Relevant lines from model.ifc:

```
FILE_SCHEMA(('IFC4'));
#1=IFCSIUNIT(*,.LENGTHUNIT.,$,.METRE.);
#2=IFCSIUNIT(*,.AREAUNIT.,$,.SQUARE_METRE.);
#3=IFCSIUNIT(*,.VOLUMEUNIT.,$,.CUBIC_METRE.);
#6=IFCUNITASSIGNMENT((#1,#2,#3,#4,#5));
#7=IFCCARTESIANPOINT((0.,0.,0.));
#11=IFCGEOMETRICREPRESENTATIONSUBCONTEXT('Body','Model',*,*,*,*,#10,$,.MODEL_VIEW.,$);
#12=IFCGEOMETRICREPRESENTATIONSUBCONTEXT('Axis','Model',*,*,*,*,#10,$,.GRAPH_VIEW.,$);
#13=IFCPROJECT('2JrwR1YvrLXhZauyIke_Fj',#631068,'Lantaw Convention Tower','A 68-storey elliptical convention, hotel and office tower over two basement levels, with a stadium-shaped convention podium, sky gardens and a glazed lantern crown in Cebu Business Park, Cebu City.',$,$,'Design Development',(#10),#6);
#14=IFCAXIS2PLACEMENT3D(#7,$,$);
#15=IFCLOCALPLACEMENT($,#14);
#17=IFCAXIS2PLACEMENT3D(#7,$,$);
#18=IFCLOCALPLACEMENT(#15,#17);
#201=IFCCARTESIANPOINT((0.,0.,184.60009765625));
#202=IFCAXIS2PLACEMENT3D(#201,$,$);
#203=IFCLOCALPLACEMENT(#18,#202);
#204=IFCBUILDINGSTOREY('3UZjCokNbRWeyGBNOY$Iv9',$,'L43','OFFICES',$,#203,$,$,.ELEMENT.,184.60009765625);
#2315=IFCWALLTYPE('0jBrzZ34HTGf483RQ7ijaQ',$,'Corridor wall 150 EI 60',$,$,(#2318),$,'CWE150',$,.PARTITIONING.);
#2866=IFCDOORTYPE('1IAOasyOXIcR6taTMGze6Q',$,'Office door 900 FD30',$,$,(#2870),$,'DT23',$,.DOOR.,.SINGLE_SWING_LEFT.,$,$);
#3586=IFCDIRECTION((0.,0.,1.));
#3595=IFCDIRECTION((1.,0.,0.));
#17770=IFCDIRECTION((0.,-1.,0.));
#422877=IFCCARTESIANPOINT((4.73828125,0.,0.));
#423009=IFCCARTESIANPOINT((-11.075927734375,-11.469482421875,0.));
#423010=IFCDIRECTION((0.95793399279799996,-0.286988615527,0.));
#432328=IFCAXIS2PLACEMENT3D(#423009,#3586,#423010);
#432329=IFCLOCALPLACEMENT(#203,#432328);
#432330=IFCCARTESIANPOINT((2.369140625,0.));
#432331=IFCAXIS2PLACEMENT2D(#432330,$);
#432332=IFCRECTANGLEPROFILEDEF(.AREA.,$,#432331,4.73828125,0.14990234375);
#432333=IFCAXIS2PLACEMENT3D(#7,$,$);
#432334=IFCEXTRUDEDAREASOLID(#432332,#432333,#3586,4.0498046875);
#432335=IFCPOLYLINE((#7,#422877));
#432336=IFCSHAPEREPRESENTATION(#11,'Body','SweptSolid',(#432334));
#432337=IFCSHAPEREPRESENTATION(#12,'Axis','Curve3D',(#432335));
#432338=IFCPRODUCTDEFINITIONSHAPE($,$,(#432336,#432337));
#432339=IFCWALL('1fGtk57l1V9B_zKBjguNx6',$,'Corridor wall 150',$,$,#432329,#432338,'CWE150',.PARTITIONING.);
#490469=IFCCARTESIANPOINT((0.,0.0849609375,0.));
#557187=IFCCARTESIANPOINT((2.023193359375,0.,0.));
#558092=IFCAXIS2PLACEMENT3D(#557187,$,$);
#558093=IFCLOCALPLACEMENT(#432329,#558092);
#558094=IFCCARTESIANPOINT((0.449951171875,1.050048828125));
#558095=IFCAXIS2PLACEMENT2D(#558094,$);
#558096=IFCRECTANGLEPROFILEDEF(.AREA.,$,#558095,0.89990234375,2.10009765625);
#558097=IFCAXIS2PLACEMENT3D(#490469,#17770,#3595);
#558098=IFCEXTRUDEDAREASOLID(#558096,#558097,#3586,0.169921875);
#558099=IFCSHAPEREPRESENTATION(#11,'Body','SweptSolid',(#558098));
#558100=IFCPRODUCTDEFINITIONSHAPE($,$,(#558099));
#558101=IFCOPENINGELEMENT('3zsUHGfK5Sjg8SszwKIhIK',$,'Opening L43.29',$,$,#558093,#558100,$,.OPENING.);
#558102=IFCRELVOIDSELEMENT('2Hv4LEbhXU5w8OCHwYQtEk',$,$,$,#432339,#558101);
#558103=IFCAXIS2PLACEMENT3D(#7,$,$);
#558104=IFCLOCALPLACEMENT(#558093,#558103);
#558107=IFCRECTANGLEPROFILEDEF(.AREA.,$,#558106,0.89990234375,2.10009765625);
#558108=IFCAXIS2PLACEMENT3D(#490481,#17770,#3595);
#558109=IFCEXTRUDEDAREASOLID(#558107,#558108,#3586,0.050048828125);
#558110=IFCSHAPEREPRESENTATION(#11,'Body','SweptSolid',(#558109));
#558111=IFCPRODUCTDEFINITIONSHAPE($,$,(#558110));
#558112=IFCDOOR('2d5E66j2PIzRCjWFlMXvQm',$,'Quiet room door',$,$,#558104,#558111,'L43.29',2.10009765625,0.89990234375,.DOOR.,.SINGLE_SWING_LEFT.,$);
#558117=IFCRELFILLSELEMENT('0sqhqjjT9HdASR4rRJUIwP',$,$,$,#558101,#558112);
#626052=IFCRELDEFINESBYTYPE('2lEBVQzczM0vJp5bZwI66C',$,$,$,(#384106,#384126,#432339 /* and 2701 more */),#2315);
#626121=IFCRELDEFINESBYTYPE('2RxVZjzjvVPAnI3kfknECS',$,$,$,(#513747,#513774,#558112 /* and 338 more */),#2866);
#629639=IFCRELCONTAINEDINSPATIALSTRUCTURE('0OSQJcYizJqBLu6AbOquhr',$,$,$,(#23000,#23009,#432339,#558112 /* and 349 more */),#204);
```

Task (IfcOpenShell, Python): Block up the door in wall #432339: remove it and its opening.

```python
import ifcopenshell
import ifcopenshell.api.feature
import ifcopenshell.api.root
import ifcopenshell.geom
import ifcopenshell.util.shape

model = ifcopenshell.open("model.ifc")
settings = ifcopenshell.geom.settings()


def volume(element):
    """Net volume in cubic metres, openings subtracted."""
    shape = ifcopenshell.geom.create_shape(settings, element)
    return ifcopenshell.util.shape.get_volume(shape.geometry)


door = model.by_guid("2d5E66j2PIzRCjWFlMXvQm")
opening = door.FillsVoids[0].RelatingOpeningElement
wall = opening.VoidsElements[0].RelatingBuildingElement
before = volume(wall)

ifcopenshell.api.root.remove_product(model, product=door)
ifcopenshell.api.feature.remove_feature(model, feature=opening)

after = volume(wall)

print(f"wall volume {before:.3f} -> {after:.3f} m3")

model.write("model_rev.ifc")
```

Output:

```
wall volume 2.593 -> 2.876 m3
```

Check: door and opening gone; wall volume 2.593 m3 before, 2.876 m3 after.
